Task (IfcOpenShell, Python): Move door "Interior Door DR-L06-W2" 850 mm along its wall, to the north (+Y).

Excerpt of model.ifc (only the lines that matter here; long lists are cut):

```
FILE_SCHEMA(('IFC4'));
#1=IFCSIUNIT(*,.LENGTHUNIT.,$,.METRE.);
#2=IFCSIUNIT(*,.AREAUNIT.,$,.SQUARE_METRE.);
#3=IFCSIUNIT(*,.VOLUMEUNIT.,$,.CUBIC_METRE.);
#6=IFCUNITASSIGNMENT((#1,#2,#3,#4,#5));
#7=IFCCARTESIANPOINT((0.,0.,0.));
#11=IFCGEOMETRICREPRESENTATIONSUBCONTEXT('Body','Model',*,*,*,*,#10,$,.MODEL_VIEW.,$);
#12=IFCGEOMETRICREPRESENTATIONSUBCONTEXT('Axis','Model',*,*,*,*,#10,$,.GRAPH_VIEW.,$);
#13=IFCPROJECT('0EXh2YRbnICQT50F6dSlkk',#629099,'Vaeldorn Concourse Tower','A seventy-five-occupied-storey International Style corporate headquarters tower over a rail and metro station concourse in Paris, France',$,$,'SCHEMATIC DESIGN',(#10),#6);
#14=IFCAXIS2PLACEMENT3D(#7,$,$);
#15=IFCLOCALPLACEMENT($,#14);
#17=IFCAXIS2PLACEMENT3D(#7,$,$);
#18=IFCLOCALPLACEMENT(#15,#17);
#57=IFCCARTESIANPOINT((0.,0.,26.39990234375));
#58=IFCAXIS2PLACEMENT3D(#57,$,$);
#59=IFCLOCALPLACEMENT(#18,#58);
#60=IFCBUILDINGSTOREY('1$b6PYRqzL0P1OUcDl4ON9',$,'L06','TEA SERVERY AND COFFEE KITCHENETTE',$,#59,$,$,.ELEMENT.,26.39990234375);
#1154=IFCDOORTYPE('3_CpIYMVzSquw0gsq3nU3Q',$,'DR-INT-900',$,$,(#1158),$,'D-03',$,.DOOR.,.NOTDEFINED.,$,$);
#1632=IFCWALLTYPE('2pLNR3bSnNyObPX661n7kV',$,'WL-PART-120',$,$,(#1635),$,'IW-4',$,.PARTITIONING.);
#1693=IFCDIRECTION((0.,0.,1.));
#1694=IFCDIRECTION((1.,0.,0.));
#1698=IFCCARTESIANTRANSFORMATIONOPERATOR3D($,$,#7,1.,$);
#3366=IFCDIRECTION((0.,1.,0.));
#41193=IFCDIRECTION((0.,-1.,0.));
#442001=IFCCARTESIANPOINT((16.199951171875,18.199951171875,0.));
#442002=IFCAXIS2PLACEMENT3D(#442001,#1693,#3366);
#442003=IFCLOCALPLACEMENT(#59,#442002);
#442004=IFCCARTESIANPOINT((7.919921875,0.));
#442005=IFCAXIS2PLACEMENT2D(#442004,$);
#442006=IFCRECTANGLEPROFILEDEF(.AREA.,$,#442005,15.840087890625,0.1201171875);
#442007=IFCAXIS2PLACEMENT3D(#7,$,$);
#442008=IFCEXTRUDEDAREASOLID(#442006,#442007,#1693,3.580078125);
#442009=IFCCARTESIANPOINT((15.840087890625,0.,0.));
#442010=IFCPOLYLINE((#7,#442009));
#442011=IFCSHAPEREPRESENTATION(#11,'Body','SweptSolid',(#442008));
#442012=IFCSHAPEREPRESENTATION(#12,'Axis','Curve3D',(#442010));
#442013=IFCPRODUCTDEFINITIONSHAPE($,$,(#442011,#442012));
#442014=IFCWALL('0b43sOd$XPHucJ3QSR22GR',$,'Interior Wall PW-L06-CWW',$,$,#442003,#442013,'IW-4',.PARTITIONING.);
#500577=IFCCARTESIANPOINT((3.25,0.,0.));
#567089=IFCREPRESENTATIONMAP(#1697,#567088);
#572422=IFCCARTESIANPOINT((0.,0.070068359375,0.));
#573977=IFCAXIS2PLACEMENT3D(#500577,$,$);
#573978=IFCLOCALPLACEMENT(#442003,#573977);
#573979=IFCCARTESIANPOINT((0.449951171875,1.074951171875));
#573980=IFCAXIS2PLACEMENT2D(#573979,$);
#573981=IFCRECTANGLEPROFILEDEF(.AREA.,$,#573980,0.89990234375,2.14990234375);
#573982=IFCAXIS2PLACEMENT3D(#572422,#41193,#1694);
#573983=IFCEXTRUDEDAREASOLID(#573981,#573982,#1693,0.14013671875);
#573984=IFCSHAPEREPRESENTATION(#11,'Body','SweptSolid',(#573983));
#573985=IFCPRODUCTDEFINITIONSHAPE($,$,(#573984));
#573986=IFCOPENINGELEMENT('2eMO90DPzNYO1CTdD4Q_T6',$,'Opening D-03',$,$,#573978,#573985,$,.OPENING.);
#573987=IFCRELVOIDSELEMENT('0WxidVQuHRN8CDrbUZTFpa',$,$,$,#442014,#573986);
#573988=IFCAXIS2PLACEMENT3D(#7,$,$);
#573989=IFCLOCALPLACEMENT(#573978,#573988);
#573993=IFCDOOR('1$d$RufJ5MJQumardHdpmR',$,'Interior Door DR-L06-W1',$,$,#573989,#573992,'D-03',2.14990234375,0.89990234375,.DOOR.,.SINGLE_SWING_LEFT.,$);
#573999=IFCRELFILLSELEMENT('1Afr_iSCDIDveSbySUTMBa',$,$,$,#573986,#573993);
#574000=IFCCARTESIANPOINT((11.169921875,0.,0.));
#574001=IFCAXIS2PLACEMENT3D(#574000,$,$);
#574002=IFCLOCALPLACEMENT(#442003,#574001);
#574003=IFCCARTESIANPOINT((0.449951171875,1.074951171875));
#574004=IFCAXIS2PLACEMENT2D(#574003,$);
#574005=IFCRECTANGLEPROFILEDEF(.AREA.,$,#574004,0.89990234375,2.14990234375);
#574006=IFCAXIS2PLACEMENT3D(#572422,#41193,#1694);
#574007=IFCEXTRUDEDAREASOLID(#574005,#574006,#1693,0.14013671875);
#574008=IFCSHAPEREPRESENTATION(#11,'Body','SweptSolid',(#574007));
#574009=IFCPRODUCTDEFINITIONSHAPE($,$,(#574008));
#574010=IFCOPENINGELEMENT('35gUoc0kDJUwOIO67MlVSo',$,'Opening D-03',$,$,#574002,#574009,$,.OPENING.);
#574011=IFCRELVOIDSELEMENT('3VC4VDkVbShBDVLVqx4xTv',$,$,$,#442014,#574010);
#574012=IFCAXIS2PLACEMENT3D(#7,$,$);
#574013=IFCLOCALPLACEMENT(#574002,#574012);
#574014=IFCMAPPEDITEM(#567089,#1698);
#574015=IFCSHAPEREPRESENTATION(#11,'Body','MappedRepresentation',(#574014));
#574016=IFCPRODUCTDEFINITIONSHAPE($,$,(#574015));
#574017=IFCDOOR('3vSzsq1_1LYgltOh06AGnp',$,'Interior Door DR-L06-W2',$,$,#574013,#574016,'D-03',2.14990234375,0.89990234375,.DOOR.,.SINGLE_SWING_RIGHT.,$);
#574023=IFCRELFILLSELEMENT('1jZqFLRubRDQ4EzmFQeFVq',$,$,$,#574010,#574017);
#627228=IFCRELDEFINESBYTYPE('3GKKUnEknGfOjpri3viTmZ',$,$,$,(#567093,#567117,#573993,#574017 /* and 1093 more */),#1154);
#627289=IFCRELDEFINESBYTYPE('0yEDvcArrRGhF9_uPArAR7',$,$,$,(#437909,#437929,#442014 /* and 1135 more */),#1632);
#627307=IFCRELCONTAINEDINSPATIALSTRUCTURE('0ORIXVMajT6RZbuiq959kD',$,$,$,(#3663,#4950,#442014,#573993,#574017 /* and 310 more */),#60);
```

```python
import ifcopenshell
import ifcopenshell.api.geometry
import ifcopenshell.util.placement

model = ifcopenshell.open("model.ifc")

door = model.by_guid("3vSzsq1_1LYgltOh06AGnp")
opening = door.FillsVoids[0].RelatingOpeningElement
wall = opening.VoidsElements[0].RelatingBuildingElement

wall_matrix = ifcopenshell.util.placement.get_local_placement(wall.ObjectPlacement)
shift = wall_matrix[:3, 0] * 0.85
before = ifcopenshell.util.placement.get_local_placement(door.ObjectPlacement)[:3, 3].copy()

# The door is placed relative to its opening, so it follows when the opening moves.
matrix = ifcopenshell.util.placement.get_local_placement(opening.ObjectPlacement)
matrix[:3, 3] += shift
ifcopenshell.api.geometry.edit_object_placement(
    model, product=opening, matrix=matrix, is_si=False, should_transform_children=True
)

after = ifcopenshell.util.placement.get_local_placement(door.ObjectPlacement)[:3, 3]
print("door moved by", (after - before).round(3) + 0.0)

model.write("model_v2.ifc")
```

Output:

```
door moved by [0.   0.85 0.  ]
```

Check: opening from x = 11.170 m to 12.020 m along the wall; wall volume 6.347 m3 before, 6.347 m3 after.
